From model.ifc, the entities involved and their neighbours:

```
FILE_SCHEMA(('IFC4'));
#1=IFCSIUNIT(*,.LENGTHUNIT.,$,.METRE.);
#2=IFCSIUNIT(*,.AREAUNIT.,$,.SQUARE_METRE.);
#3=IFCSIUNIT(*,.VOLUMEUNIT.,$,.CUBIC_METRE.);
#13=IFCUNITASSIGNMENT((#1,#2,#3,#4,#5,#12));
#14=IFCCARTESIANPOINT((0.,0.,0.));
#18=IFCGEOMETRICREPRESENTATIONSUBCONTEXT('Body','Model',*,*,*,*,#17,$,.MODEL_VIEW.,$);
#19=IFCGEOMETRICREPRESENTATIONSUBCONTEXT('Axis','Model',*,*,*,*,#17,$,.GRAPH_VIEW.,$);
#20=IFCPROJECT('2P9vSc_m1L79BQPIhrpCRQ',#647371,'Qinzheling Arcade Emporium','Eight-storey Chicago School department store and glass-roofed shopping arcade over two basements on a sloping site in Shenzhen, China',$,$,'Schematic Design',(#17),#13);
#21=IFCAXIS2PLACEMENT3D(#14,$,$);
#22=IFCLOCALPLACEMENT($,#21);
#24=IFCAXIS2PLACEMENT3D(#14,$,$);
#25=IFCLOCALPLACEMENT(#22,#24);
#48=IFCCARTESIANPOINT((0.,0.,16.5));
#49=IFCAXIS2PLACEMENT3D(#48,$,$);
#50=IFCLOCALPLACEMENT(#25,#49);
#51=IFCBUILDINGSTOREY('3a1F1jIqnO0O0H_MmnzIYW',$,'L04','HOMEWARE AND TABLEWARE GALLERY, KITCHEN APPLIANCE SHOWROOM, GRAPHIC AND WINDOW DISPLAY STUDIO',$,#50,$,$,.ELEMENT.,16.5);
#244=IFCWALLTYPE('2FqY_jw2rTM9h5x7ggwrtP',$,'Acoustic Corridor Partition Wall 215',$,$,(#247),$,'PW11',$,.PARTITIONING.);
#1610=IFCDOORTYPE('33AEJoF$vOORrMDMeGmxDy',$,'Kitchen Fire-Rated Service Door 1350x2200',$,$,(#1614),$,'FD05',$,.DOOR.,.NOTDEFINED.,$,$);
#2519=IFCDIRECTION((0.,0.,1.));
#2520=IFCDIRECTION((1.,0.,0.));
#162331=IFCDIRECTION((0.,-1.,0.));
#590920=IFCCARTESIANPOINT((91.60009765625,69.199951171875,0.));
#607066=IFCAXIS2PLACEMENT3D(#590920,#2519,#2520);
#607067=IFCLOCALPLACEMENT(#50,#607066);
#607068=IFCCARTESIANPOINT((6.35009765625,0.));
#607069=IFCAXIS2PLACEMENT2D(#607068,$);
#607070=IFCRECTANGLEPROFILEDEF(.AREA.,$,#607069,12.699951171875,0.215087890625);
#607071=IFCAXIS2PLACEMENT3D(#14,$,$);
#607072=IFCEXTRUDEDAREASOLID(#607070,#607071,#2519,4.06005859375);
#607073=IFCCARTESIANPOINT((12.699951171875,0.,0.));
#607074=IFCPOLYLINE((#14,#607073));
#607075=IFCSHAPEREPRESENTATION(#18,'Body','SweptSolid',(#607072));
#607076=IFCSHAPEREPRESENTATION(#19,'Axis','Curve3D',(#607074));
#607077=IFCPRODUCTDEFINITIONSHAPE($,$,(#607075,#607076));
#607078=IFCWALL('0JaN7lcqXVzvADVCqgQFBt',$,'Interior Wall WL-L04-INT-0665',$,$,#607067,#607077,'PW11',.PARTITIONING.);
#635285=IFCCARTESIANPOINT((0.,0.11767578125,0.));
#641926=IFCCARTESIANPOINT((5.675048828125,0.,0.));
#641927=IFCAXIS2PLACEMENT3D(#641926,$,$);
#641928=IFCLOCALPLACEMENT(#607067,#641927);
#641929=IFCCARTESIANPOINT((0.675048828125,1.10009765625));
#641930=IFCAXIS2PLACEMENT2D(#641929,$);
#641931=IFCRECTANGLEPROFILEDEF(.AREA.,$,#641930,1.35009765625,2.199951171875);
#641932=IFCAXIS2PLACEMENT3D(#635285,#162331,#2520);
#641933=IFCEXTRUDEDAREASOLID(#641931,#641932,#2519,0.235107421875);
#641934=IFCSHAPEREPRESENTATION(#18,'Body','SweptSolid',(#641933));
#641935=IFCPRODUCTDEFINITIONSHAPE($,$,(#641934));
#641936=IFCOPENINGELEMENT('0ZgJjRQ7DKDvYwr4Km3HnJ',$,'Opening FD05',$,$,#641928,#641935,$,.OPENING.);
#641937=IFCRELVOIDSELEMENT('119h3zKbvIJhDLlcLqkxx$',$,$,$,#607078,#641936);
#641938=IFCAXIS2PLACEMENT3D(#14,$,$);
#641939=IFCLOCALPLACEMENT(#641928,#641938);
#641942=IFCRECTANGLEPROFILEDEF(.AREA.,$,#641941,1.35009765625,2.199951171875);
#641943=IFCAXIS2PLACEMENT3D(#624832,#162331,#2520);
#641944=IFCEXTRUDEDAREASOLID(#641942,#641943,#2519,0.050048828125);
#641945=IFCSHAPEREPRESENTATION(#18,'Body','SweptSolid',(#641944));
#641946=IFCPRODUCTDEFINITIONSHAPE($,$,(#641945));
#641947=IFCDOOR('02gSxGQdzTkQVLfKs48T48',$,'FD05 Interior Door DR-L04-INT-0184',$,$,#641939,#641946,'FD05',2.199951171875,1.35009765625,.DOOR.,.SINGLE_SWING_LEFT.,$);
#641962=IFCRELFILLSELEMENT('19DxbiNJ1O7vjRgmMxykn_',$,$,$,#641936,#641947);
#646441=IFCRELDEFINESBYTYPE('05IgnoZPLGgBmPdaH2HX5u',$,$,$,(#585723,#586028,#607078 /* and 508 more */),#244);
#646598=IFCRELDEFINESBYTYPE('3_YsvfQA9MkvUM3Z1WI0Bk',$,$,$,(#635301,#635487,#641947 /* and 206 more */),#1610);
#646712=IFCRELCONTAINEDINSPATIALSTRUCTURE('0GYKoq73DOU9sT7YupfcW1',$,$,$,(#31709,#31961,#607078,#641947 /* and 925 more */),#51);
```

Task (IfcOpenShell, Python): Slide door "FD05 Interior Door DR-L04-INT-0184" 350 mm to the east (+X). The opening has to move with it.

```python
import ifcopenshell
import ifcopenshell.api.geometry
import ifcopenshell.util.placement
import ifcopenshell.util.unit

model = ifcopenshell.open("model.ifc")
unit_scale = ifcopenshell.util.unit.calculate_unit_scale(model)

door = model.by_guid("02gSxGQdzTkQVLfKs48T48")
opening = door.FillsVoids[0].RelatingOpeningElement
wall = opening.VoidsElements[0].RelatingBuildingElement

wall_matrix = ifcopenshell.util.placement.get_local_placement(wall.ObjectPlacement)
shift = wall_matrix[:3, 0] * 0.35 / unit_scale
before = ifcopenshell.util.placement.get_local_placement(door.ObjectPlacement)[:3, 3].copy()

# The door is placed relative to its opening, so it follows when the opening moves.
matrix = ifcopenshell.util.placement.get_local_placement(opening.ObjectPlacement)
matrix[:3, 3] += shift
ifcopenshell.api.geometry.edit_object_placement(
    model, product=opening, matrix=matrix, is_si=False, should_transform_children=True
)

after = ifcopenshell.util.placement.get_local_placement(door.ObjectPlacement)[:3, 3]
print("door moved by", (after - before).round(3) + 0.0)

model.write("model_edited.ifc")
```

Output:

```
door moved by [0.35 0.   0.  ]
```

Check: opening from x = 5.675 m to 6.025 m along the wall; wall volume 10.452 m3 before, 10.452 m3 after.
